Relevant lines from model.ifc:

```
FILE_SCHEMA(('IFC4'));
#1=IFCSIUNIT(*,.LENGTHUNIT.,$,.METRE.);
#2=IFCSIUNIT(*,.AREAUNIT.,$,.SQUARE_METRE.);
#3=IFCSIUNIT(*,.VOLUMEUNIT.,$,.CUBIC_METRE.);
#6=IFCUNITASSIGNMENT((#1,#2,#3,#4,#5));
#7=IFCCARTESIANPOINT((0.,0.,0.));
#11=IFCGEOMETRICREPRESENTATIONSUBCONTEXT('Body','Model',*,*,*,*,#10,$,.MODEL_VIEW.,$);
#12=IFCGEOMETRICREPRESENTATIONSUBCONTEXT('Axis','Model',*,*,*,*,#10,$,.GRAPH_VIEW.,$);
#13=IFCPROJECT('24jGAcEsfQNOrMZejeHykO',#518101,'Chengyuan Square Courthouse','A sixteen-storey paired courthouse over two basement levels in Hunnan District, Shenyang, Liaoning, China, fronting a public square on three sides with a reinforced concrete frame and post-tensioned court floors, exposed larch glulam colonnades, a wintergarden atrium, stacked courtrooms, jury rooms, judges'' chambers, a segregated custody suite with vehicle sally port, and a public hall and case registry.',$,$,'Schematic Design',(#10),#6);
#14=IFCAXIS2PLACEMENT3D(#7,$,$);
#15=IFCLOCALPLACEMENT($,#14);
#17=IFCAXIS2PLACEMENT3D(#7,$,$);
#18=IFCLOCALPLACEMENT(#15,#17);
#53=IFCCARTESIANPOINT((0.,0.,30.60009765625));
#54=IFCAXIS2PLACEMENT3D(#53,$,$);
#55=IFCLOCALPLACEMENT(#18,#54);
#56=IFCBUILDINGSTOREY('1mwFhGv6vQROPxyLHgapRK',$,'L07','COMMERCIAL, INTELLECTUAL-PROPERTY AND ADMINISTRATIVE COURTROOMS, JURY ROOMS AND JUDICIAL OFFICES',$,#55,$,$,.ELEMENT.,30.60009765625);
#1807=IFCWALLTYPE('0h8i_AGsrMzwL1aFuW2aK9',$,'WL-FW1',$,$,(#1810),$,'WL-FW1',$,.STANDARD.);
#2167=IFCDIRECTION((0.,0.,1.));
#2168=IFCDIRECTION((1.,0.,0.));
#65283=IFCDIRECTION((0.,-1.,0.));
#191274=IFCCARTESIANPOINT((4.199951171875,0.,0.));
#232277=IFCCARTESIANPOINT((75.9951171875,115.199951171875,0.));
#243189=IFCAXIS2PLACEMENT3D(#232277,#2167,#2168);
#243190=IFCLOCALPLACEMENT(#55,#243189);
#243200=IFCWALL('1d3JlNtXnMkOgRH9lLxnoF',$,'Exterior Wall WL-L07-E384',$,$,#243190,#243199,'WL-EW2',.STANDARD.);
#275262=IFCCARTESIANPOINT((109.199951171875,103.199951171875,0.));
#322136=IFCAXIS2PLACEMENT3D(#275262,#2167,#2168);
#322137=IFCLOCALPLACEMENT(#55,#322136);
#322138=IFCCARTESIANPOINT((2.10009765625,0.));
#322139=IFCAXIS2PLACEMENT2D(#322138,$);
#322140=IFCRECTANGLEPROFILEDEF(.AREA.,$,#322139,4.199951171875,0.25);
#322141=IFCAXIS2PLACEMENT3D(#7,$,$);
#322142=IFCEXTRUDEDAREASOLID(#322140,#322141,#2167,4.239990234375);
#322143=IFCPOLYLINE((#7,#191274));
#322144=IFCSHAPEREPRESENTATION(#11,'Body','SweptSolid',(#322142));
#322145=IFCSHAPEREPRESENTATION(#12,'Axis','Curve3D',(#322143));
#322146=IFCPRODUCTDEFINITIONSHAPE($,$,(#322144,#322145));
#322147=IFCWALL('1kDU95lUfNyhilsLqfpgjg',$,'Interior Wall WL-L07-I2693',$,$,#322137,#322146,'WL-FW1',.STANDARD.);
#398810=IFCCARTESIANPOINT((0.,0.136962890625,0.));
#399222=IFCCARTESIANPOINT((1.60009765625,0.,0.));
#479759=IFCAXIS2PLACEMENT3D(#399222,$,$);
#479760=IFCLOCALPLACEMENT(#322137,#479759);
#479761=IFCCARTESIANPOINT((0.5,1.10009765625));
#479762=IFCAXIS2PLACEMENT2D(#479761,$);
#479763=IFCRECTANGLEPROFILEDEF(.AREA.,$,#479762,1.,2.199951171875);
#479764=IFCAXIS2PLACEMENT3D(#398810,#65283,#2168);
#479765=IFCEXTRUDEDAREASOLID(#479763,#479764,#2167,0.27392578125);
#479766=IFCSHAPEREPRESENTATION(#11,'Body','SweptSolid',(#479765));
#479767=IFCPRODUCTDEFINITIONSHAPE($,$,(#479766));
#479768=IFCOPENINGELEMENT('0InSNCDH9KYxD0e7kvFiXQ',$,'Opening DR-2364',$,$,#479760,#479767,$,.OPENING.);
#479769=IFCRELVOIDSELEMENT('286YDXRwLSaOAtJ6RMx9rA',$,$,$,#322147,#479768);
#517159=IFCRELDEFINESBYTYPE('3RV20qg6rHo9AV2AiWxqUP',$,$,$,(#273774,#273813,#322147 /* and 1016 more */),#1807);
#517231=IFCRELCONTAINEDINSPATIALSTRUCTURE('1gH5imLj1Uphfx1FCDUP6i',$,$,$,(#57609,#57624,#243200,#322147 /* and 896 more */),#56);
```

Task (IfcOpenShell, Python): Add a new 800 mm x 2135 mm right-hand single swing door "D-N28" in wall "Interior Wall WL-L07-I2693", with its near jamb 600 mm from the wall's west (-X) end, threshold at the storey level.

```python
import numpy as np
import ifcopenshell
import ifcopenshell.api.feature
import ifcopenshell.api.geometry
import ifcopenshell.api.root
import ifcopenshell.api.spatial
import ifcopenshell.geom
import ifcopenshell.util.element
import ifcopenshell.util.placement
import ifcopenshell.util.representation
import ifcopenshell.util.shape
import ifcopenshell.util.unit

model = ifcopenshell.open("model.ifc")
unit_scale = ifcopenshell.util.unit.calculate_unit_scale(model)
settings = ifcopenshell.geom.settings()


def volume(element):
    """Net volume in cubic metres, openings subtracted."""
    shape = ifcopenshell.geom.create_shape(settings, element)
    return ifcopenshell.util.shape.get_volume(shape.geometry)


wall = model.by_id(322147)
storey = ifcopenshell.util.element.get_container(wall, ifc_class="IfcBuildingStorey")
context = ifcopenshell.util.representation.get_context(model, "Model", "Body", "MODEL_VIEW")
before = volume(wall)

width, height, from_end, sill = 0.8, 2.135, 0.6, 0.0  # metres

# The wall runs along its own X axis, and the end named is its -X end.
wall_shape = ifcopenshell.geom.create_shape(settings, wall)
x, y, z = ifcopenshell.util.shape.get_vertices(wall_shape.geometry).T
start = x.min() + from_end
face, thickness = float(y.min()), float(y.max() - y.min())
wall_matrix = ifcopenshell.util.placement.get_local_placement(wall.ObjectPlacement)
level = ifcopenshell.util.placement.get_local_placement(storey.ObjectPlacement)[2, 3]


def in_wall(x, y):
    """Placement at x, y metres in the wall's axes, at sill height."""
    matrix = wall_matrix.copy()
    matrix[:, 3] = wall_matrix @ np.array([x / unit_scale, y / unit_scale, 0.0, 1.0])
    matrix[2, 3] = level + sill / unit_scale
    return matrix


# Opening: a box that overshoots both wall faces by 50 mm.
opening = ifcopenshell.api.root.create_entity(model, ifc_class="IfcOpeningElement", predefined_type="OPENING")
box = ifcopenshell.api.geometry.add_wall_representation(
    model, context=context, length=width, height=height, thickness=thickness + 0.1
)
ifcopenshell.api.geometry.assign_representation(model, product=opening, representation=box)
ifcopenshell.api.geometry.edit_object_placement(model, product=opening, matrix=in_wall(start, face - 0.05), is_si=False)
ifcopenshell.api.feature.add_feature(model, feature=opening, element=wall)

door = ifcopenshell.api.root.create_entity(model, ifc_class="IfcDoor", name="D-N28", predefined_type="DOOR")
door.OverallWidth, door.OverallHeight = width / unit_scale, height / unit_scale
door.OperationType = "SINGLE_SWING_RIGHT"
body = ifcopenshell.api.geometry.add_door_representation(
    model,
    context=context,
    overall_width=door.OverallWidth,
    overall_height=door.OverallHeight,
    operation_type="SINGLE_SWING_RIGHT",
    lining_properties={"LiningDepth": thickness / unit_scale, "ThresholdDepth": thickness / unit_scale},
)
ifcopenshell.api.geometry.assign_representation(model, product=door, representation=body)
ifcopenshell.api.spatial.assign_container(model, products=[door], relating_structure=storey)
ifcopenshell.api.feature.add_filling(model, opening=opening, element=door)

# The lining spans the wall, so the door starts at the wall face.
ifcopenshell.api.geometry.edit_object_placement(model, product=door, matrix=in_wall(start, face), is_si=False)

after = volume(wall)

print(f"wall volume {before:.3f} -> {after:.3f} m3")

model.write("model_v2.ifc")
```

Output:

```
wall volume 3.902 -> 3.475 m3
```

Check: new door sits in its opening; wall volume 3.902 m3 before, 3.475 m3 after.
